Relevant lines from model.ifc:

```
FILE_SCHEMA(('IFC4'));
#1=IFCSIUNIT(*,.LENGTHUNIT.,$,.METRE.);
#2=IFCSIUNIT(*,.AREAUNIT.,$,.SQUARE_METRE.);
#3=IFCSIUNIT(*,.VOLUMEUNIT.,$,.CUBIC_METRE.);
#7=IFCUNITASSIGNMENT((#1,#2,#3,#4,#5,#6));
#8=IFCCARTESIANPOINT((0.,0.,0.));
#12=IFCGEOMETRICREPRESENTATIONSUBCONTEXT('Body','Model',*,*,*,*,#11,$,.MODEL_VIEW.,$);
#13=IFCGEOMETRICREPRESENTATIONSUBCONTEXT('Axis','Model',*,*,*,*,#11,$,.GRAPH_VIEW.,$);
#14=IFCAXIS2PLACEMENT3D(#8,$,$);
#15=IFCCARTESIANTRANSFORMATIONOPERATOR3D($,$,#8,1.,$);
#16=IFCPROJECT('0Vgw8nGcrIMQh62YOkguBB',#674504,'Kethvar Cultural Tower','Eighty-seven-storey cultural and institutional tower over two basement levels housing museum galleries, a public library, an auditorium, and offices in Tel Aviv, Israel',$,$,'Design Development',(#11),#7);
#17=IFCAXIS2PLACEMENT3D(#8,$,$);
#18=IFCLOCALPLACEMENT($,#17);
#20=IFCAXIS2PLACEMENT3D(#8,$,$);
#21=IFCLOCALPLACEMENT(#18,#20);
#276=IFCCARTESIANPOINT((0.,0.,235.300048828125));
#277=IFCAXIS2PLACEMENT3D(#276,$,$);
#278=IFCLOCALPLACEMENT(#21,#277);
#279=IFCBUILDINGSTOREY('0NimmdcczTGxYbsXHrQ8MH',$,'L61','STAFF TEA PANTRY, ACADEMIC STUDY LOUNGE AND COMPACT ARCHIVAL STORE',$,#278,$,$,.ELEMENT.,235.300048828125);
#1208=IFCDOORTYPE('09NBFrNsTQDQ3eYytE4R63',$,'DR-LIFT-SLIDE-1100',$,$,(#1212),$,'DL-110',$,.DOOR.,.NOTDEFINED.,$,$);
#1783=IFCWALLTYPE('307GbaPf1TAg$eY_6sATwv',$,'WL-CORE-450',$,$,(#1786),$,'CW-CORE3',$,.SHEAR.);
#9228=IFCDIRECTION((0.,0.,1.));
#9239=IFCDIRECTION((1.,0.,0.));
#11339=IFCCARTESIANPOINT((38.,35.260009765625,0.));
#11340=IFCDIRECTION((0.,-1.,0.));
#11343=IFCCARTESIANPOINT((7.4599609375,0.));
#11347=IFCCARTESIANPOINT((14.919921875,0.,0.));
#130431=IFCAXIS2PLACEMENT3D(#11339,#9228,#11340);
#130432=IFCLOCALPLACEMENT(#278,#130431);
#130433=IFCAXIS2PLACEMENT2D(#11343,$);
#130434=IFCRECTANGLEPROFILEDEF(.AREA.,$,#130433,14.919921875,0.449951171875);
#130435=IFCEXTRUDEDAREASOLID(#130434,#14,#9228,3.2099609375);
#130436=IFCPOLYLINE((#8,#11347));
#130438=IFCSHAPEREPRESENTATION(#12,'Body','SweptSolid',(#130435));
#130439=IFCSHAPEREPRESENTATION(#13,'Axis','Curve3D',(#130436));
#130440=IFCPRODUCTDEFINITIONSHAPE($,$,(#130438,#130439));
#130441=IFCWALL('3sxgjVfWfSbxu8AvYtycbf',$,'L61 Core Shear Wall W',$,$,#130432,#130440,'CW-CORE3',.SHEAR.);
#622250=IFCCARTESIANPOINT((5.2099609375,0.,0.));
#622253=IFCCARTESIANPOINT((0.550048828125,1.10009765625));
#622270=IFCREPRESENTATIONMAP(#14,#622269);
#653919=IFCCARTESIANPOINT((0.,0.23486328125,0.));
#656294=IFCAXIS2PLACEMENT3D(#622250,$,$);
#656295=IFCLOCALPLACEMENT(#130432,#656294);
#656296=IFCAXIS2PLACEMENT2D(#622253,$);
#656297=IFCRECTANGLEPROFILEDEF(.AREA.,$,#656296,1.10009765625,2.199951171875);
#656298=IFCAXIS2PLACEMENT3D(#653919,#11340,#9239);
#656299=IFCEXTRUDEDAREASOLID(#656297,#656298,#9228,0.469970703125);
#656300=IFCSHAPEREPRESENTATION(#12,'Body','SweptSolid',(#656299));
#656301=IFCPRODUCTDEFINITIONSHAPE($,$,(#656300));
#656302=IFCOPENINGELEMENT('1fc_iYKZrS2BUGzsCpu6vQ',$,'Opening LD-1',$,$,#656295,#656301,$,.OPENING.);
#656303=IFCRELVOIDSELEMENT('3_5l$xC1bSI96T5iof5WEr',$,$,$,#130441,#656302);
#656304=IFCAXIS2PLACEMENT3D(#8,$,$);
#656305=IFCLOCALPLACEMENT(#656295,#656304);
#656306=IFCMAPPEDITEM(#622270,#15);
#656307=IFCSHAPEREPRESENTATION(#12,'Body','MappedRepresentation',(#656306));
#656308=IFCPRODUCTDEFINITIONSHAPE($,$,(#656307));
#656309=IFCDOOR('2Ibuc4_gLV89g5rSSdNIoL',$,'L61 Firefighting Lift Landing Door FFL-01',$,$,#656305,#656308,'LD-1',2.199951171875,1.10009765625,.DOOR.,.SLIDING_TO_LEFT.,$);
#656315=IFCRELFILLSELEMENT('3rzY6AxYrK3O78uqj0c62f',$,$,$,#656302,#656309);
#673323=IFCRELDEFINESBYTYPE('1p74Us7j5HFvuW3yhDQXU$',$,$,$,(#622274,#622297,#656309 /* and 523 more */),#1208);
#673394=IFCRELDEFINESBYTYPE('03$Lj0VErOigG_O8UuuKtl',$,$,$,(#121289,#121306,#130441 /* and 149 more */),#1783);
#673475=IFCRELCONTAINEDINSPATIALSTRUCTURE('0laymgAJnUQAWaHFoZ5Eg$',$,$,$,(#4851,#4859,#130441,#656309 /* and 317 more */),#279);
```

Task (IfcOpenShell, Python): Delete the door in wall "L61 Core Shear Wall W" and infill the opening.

```python
import ifcopenshell
import ifcopenshell.api.feature
import ifcopenshell.api.root
import ifcopenshell.geom
import ifcopenshell.util.shape

model = ifcopenshell.open("model.ifc")
settings = ifcopenshell.geom.settings()


def volume(element):
    """Net volume in cubic metres, openings subtracted."""
    shape = ifcopenshell.geom.create_shape(settings, element)
    return ifcopenshell.util.shape.get_volume(shape.geometry)


door = model.by_guid("2Ibuc4_gLV89g5rSSdNIoL")
opening = door.FillsVoids[0].RelatingOpeningElement
wall = opening.VoidsElements[0].RelatingBuildingElement
before = volume(wall)

ifcopenshell.api.root.remove_product(model, product=door)
ifcopenshell.api.feature.remove_feature(model, feature=opening)

after = volume(wall)

print(f"wall volume {before:.3f} -> {after:.3f} m3")

model.write("model_updated.ifc")
```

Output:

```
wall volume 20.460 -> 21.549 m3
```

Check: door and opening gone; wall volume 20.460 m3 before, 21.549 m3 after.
